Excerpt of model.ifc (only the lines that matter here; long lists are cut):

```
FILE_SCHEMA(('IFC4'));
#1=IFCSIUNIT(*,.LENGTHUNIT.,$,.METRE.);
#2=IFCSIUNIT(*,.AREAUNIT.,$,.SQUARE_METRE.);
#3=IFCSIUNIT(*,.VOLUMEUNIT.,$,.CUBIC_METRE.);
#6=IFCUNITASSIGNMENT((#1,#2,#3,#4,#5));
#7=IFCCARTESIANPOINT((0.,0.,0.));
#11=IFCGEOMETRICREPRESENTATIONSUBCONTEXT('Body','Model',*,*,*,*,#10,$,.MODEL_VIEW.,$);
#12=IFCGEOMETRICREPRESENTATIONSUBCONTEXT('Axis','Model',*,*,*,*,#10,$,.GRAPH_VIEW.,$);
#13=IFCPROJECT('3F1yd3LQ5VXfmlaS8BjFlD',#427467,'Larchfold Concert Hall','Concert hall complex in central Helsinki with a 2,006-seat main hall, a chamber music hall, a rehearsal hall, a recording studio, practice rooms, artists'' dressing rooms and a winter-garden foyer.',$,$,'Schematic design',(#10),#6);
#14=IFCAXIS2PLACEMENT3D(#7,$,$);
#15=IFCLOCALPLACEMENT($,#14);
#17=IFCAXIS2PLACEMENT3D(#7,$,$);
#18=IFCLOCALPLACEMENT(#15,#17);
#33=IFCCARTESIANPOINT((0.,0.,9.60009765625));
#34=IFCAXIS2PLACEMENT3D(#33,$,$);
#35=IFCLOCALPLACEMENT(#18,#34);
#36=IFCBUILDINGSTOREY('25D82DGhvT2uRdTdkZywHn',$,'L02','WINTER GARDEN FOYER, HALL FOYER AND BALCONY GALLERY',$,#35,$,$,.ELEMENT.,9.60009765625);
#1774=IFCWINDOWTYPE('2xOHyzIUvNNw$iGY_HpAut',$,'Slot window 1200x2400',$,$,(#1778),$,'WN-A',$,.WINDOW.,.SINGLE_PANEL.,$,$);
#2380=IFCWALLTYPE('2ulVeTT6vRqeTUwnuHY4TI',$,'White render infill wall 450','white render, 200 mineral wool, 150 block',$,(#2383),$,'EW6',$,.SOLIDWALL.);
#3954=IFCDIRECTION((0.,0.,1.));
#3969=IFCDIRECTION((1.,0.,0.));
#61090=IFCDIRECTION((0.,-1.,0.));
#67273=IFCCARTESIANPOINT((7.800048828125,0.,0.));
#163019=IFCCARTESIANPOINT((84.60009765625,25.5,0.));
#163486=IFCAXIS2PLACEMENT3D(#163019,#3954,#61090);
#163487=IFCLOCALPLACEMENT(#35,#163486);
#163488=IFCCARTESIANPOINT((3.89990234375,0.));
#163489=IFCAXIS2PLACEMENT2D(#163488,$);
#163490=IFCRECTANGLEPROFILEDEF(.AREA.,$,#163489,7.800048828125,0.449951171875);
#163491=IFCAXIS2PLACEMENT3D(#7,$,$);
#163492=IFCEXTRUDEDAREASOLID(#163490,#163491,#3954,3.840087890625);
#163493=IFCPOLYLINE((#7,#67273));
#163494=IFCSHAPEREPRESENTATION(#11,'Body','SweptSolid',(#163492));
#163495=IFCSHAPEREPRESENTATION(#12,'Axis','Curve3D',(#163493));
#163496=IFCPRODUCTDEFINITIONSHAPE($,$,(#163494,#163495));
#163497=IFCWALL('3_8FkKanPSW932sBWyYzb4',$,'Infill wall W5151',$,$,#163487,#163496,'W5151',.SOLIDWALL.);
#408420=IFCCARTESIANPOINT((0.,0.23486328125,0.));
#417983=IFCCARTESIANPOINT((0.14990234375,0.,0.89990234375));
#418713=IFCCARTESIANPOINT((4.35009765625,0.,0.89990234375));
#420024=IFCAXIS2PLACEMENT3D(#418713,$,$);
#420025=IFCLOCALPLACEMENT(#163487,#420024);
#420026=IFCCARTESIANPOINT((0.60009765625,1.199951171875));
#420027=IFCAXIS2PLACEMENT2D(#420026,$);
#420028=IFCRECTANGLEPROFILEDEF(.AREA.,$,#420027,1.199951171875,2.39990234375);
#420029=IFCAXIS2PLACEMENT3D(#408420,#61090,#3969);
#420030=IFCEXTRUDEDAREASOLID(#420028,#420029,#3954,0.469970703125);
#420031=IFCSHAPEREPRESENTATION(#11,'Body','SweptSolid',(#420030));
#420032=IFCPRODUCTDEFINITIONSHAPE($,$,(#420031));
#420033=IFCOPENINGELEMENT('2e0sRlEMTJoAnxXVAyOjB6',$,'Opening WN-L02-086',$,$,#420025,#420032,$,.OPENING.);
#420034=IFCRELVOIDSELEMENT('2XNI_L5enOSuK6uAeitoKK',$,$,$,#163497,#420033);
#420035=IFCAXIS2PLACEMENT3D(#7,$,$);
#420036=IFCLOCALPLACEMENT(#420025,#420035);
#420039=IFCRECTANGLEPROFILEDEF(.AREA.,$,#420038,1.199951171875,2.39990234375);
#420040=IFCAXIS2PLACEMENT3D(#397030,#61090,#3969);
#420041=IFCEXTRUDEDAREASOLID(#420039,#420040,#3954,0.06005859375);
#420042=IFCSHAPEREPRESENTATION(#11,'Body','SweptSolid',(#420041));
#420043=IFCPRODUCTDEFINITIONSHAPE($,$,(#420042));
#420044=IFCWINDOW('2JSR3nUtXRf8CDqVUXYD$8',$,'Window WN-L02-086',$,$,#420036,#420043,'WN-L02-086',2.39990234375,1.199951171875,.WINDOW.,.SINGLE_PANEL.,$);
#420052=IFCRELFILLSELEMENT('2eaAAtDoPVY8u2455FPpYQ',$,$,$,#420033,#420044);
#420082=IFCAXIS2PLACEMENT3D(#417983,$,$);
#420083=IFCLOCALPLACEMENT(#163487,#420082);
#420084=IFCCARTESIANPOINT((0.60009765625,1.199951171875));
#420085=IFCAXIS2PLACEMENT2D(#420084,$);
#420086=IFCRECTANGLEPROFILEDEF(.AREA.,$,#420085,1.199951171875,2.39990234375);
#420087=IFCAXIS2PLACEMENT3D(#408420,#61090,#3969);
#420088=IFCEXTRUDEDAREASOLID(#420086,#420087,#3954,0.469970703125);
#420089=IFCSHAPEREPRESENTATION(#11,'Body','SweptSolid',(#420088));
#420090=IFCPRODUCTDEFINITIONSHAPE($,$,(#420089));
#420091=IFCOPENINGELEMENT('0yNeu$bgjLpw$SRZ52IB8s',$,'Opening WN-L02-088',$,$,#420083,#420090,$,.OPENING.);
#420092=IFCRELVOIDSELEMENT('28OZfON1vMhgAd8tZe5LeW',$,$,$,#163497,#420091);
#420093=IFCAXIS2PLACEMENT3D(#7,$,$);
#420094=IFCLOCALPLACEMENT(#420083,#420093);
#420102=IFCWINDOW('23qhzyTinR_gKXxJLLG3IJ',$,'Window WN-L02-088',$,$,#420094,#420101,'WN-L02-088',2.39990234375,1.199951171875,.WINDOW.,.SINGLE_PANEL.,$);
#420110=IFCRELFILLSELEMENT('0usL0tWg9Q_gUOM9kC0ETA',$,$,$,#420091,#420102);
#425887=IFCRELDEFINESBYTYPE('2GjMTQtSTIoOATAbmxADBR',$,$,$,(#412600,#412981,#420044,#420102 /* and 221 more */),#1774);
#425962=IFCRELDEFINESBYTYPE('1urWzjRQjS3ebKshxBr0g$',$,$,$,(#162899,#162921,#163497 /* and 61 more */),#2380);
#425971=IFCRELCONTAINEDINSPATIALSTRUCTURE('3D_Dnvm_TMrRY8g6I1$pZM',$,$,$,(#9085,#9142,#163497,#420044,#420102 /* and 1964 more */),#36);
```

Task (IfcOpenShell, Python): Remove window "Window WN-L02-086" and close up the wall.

```python
import ifcopenshell
import ifcopenshell.api.feature
import ifcopenshell.api.root
import ifcopenshell.geom
import ifcopenshell.util.shape

model = ifcopenshell.open("model.ifc")
settings = ifcopenshell.geom.settings()


def volume(element):
    """Net volume in cubic metres, openings subtracted."""
    shape = ifcopenshell.geom.create_shape(settings, element)
    return ifcopenshell.util.shape.get_volume(shape.geometry)


window = model.by_guid("2JSR3nUtXRf8CDqVUXYD$8")
opening = window.FillsVoids[0].RelatingOpeningElement
wall = opening.VoidsElements[0].RelatingBuildingElement
before = volume(wall)

ifcopenshell.api.root.remove_product(model, product=window)
ifcopenshell.api.feature.remove_feature(model, feature=opening)

after = volume(wall)

print(f"wall volume {before:.3f} -> {after:.3f} m3")

model.write("model_rev.ifc")
```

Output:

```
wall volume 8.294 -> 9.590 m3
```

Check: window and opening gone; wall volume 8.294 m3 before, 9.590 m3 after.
